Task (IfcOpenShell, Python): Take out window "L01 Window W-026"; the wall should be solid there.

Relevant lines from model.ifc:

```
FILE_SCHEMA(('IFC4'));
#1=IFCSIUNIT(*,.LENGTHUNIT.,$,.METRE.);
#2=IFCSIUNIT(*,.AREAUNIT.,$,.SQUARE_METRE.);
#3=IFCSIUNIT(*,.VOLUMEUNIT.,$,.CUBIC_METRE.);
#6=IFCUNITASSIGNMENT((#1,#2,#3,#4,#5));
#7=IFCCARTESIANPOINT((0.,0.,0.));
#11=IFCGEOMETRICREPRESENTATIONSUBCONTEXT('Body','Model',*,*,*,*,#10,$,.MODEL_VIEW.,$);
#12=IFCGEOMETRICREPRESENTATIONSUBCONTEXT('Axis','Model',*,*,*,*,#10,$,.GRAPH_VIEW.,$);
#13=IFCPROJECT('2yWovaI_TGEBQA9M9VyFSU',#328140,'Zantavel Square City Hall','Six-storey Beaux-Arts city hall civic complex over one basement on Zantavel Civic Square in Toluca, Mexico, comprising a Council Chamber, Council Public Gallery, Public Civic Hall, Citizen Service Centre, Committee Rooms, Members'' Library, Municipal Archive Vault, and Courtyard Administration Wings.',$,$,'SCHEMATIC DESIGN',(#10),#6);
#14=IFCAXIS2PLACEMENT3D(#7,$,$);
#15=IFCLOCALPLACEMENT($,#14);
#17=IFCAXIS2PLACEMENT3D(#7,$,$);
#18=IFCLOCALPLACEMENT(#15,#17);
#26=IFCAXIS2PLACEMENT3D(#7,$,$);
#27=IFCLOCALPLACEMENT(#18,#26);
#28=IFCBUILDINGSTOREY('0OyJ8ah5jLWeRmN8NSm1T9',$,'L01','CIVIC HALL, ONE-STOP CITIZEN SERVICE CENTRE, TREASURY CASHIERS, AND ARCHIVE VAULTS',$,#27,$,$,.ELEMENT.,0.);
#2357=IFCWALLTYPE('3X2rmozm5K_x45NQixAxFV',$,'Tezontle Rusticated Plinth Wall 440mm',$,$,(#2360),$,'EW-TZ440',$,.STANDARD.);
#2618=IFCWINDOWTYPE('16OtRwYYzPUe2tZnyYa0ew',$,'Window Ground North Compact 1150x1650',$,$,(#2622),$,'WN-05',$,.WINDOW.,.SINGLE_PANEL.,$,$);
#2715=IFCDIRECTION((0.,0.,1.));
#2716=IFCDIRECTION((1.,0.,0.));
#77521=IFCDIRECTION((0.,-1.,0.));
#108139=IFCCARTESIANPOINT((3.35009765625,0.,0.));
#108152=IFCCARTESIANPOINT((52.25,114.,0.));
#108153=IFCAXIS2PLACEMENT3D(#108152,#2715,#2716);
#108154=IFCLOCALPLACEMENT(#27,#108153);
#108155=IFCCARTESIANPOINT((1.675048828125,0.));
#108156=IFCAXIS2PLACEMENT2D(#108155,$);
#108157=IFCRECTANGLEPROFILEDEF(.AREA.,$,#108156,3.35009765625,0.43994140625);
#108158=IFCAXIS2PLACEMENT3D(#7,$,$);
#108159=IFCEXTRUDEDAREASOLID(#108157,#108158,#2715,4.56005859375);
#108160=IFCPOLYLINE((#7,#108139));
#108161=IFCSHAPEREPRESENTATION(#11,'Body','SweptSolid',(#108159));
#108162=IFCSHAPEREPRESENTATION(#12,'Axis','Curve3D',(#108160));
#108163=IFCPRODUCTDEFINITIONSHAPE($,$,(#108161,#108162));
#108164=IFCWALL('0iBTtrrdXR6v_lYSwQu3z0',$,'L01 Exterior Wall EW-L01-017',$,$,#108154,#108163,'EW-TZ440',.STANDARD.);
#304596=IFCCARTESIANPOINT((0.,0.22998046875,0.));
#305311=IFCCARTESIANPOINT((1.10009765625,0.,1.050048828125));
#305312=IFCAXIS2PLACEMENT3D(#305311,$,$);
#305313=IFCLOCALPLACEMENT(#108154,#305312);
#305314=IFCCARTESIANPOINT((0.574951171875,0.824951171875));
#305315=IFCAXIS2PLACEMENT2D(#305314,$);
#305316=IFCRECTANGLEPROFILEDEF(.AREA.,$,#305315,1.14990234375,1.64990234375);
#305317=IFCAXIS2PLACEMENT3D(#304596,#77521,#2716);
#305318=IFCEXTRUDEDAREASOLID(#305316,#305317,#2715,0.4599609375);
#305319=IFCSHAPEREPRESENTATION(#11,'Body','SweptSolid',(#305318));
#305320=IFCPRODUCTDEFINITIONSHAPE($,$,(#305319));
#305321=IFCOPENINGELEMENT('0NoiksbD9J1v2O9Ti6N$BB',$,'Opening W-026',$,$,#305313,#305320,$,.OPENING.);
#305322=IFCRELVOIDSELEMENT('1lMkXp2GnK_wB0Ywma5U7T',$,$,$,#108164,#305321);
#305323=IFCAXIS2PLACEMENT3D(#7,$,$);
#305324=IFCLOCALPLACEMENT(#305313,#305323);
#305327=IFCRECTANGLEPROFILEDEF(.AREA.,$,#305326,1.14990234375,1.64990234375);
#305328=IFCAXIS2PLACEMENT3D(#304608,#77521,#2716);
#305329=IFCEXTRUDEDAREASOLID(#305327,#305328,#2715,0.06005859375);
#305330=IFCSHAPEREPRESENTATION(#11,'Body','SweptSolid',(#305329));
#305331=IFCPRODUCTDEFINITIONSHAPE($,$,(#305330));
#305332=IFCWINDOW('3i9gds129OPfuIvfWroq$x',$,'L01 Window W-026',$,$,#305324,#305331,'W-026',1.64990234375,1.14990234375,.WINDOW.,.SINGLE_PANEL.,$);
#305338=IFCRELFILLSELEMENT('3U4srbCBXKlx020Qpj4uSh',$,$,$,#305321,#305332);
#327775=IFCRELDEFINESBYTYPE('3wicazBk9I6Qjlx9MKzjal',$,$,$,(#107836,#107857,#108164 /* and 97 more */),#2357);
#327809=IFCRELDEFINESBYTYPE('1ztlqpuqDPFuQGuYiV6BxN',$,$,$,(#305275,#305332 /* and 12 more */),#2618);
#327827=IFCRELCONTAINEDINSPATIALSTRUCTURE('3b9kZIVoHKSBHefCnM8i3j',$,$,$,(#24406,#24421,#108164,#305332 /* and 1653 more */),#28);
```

```python
import ifcopenshell
import ifcopenshell.api.feature
import ifcopenshell.api.root
import ifcopenshell.geom
import ifcopenshell.util.shape

model = ifcopenshell.open("model.ifc")
settings = ifcopenshell.geom.settings()


def volume(element):
    """Net volume in cubic metres, openings subtracted."""
    shape = ifcopenshell.geom.create_shape(settings, element)
    return ifcopenshell.util.shape.get_volume(shape.geometry)


window = model.by_id(305332)
opening = window.FillsVoids[0].RelatingOpeningElement
wall = opening.VoidsElements[0].RelatingBuildingElement
before = volume(wall)

ifcopenshell.api.root.remove_product(model, product=window)
ifcopenshell.api.feature.remove_feature(model, feature=opening)

after = volume(wall)

print(f"wall volume {before:.3f} -> {after:.3f} m3")

model.write("model_rev.ifc")
```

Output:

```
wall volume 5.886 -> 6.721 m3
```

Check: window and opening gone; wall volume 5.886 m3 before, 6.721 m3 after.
